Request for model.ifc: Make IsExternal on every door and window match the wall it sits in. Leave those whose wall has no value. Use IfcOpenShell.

First a look at what the model holds.

```python
import ifcopenshell
import ifcopenshell.util.element

model = ifcopenshell.open("model.ifc")
print(model.schema)
seen = {}
for e in model.by_type("IfcDoor") + model.by_type("IfcWindow"):
    if not e.FillsVoids:
        continue
    host = e.FillsVoids[0].RelatingOpeningElement.VoidsElements[0].RelatingBuildingElement
    own = ifcopenshell.util.element.get_pset(e, f"Pset_{e.is_a()[3:].removesuffix('StandardCase')}Common", "IsExternal")
    wall = ifcopenshell.util.element.get_pset(host, "Pset_WallCommon", "IsExternal")
    seen[e.is_a(), own, wall] = seen.get((e.is_a(), own, wall), 0) + 1
for (cls, own, wall), count in sorted(seen.items(), key=str):
    print(count, cls, "IsExternal:", own, "| host wall:", wall)
```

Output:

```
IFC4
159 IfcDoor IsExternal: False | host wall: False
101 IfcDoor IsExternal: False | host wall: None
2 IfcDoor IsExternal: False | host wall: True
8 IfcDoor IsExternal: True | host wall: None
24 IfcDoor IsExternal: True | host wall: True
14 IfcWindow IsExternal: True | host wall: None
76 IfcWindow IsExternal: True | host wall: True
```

```python
import ifcopenshell
import ifcopenshell.api.pset
import ifcopenshell.util.element

model = ifcopenshell.open("model.ifc")

count = 0
for ifc_class, pset_name in (("IfcDoor", "Pset_DoorCommon"), ("IfcWindow", "Pset_WindowCommon")):
    for e in model.by_type(ifc_class):
        if not e.FillsVoids:
            continue
        host = e.FillsVoids[0].RelatingOpeningElement.VoidsElements[0].RelatingBuildingElement
        external = ifcopenshell.util.element.get_pset(host, "Pset_WallCommon", "IsExternal")
        if external is None or ifcopenshell.util.element.get_pset(e, pset_name, "IsExternal") == external:
            continue
        pset = ifcopenshell.api.pset.add_pset(model, product=e, name=pset_name)
        ifcopenshell.api.pset.edit_pset(model, pset=pset, properties={"IsExternal": external})
        count += 1

print(count, "updated")

model.write("model_edited.ifc")
```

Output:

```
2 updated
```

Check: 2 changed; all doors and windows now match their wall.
